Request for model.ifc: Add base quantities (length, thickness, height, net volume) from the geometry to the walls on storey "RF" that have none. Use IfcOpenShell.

First a look at what the model holds.

```python
import ifcopenshell
import ifcopenshell.util.element
import ifcopenshell.util.unit

model = ifcopenshell.open("model.ifc")
print(model.schema)
for unit_type in ("LENGTHUNIT", "AREAUNIT", "VOLUMEUNIT"):
    print(unit_type, ifcopenshell.util.unit.calculate_unit_scale(model, unit_type))
storey = next(s for s in model.by_type("IfcBuildingStorey") if s.Name == "RF")
walls = [e for e in ifcopenshell.util.element.get_decomposition(storey) if e.is_a("IfcWall")]
for e in sorted(walls, key=lambda e: e.id()):
    print(e.id(), e.is_a(), e.Name, list(ifcopenshell.util.element.get_psets(e, qtos_only=True)), sep=" | ")
```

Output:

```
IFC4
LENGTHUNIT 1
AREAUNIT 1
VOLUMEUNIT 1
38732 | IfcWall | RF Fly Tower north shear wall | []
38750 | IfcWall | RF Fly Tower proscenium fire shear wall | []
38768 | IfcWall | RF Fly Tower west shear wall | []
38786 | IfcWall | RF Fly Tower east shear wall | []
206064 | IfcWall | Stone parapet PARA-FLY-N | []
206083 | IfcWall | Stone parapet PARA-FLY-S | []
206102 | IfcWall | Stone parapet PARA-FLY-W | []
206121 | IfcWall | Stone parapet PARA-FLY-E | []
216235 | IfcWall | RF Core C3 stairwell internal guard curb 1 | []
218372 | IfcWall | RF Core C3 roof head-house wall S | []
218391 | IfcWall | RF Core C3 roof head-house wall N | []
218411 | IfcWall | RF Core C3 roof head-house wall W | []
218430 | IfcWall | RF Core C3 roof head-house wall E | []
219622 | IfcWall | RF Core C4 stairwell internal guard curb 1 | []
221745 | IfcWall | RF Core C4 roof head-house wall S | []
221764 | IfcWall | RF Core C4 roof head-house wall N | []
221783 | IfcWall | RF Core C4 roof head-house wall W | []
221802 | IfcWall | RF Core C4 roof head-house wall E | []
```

```python
import ifcopenshell
import ifcopenshell.api.pset
import ifcopenshell.geom
import ifcopenshell.util.element
import ifcopenshell.util.shape
import ifcopenshell.util.unit

model = ifcopenshell.open("model.ifc")
unit_scale = ifcopenshell.util.unit.calculate_unit_scale(model)
volume_scale = ifcopenshell.util.unit.calculate_unit_scale(model, "VOLUMEUNIT")
settings = ifcopenshell.geom.settings()

storey = next(s for s in model.by_type("IfcBuildingStorey") if s.Name == "RF")
walls = [e for e in ifcopenshell.util.element.get_decomposition(storey) if e.is_a("IfcWall")]

for e in sorted(walls, key=lambda e: e.id()):
    if ifcopenshell.util.element.get_psets(e, qtos_only=True, should_inherit=False):
        continue
    # Geometry comes back in metres, in the element's own axes.
    shape = ifcopenshell.geom.create_shape(settings, e)
    values = {
        "Length": ifcopenshell.util.shape.get_x(shape.geometry) / unit_scale,
        "Width": ifcopenshell.util.shape.get_y(shape.geometry) / unit_scale,
        "Height": ifcopenshell.util.shape.get_z(shape.geometry) / unit_scale,
        "NetVolume": ifcopenshell.util.shape.get_volume(shape.geometry) / volume_scale,
    }
    qto = ifcopenshell.api.pset.add_qto(model, product=e, name="Qto_WallBaseQuantities")
    ifcopenshell.api.pset.edit_qto(model, qto=qto, properties=values)
    print(e.id(), {k: round(v, 3) for k, v in values.items()})

model.write("model_updated.ifc")
```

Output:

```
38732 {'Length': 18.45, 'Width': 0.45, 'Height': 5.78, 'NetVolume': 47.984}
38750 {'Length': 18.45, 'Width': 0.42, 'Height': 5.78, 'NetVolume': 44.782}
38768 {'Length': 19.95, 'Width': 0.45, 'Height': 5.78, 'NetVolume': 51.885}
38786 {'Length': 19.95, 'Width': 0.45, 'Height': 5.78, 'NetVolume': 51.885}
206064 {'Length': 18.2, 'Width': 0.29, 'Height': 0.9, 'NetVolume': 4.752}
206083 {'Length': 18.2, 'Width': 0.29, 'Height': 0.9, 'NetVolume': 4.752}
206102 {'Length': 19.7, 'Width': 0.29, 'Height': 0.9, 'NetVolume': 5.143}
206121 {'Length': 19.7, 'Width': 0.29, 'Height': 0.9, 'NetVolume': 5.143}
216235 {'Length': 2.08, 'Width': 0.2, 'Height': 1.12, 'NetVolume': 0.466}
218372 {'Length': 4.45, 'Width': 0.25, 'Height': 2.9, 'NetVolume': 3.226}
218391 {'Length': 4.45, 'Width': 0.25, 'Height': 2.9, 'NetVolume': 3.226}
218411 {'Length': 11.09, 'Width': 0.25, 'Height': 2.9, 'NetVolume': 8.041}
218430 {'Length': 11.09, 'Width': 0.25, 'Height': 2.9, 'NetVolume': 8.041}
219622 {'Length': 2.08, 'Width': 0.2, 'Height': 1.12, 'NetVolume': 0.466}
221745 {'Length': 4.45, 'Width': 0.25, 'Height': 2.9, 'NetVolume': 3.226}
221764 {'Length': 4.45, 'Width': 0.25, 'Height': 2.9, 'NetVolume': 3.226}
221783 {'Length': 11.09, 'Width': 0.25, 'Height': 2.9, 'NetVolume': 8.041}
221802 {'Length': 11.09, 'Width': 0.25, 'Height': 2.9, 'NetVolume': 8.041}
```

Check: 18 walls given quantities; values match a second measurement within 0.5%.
